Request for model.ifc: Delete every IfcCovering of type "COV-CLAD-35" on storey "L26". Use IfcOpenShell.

First a look at what the model holds.

```python
import ifcopenshell
import ifcopenshell.util.element

model = ifcopenshell.open("model.ifc")
print(model.schema)
storey = next(s for s in model.by_type("IfcBuildingStorey") if s.Name == "L26")
coverings = [e for e in ifcopenshell.util.element.get_decomposition(storey) if e.is_a("IfcCovering")]
seen = {}
for e in coverings:
    element_type = ifcopenshell.util.element.get_type(e)
    name = element_type.Name if element_type not in (None, e) else None
    seen[name] = seen.get(name, 0) + 1
for name, count in sorted(seen.items(), key=str):
    print(count, "x", name)
```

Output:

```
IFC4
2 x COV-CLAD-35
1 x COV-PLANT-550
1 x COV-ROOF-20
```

```python
import ifcopenshell
import ifcopenshell.api.root
import ifcopenshell.util.element

model = ifcopenshell.open("model.ifc")

storey = next(s for s in model.by_type("IfcBuildingStorey") if s.Name == "L26")
coverings = [e for e in ifcopenshell.util.element.get_decomposition(storey) if e.is_a("IfcCovering")]
targets = [e for e in coverings if (t := ifcopenshell.util.element.get_type(e)) not in (None, e) and t.Name == "COV-CLAD-35"]

for e in targets:
    ifcopenshell.api.root.remove_product(model, product=e)
print(len(targets), "removed")

model.write("model_v2.ifc")
```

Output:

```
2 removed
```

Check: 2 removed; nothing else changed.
